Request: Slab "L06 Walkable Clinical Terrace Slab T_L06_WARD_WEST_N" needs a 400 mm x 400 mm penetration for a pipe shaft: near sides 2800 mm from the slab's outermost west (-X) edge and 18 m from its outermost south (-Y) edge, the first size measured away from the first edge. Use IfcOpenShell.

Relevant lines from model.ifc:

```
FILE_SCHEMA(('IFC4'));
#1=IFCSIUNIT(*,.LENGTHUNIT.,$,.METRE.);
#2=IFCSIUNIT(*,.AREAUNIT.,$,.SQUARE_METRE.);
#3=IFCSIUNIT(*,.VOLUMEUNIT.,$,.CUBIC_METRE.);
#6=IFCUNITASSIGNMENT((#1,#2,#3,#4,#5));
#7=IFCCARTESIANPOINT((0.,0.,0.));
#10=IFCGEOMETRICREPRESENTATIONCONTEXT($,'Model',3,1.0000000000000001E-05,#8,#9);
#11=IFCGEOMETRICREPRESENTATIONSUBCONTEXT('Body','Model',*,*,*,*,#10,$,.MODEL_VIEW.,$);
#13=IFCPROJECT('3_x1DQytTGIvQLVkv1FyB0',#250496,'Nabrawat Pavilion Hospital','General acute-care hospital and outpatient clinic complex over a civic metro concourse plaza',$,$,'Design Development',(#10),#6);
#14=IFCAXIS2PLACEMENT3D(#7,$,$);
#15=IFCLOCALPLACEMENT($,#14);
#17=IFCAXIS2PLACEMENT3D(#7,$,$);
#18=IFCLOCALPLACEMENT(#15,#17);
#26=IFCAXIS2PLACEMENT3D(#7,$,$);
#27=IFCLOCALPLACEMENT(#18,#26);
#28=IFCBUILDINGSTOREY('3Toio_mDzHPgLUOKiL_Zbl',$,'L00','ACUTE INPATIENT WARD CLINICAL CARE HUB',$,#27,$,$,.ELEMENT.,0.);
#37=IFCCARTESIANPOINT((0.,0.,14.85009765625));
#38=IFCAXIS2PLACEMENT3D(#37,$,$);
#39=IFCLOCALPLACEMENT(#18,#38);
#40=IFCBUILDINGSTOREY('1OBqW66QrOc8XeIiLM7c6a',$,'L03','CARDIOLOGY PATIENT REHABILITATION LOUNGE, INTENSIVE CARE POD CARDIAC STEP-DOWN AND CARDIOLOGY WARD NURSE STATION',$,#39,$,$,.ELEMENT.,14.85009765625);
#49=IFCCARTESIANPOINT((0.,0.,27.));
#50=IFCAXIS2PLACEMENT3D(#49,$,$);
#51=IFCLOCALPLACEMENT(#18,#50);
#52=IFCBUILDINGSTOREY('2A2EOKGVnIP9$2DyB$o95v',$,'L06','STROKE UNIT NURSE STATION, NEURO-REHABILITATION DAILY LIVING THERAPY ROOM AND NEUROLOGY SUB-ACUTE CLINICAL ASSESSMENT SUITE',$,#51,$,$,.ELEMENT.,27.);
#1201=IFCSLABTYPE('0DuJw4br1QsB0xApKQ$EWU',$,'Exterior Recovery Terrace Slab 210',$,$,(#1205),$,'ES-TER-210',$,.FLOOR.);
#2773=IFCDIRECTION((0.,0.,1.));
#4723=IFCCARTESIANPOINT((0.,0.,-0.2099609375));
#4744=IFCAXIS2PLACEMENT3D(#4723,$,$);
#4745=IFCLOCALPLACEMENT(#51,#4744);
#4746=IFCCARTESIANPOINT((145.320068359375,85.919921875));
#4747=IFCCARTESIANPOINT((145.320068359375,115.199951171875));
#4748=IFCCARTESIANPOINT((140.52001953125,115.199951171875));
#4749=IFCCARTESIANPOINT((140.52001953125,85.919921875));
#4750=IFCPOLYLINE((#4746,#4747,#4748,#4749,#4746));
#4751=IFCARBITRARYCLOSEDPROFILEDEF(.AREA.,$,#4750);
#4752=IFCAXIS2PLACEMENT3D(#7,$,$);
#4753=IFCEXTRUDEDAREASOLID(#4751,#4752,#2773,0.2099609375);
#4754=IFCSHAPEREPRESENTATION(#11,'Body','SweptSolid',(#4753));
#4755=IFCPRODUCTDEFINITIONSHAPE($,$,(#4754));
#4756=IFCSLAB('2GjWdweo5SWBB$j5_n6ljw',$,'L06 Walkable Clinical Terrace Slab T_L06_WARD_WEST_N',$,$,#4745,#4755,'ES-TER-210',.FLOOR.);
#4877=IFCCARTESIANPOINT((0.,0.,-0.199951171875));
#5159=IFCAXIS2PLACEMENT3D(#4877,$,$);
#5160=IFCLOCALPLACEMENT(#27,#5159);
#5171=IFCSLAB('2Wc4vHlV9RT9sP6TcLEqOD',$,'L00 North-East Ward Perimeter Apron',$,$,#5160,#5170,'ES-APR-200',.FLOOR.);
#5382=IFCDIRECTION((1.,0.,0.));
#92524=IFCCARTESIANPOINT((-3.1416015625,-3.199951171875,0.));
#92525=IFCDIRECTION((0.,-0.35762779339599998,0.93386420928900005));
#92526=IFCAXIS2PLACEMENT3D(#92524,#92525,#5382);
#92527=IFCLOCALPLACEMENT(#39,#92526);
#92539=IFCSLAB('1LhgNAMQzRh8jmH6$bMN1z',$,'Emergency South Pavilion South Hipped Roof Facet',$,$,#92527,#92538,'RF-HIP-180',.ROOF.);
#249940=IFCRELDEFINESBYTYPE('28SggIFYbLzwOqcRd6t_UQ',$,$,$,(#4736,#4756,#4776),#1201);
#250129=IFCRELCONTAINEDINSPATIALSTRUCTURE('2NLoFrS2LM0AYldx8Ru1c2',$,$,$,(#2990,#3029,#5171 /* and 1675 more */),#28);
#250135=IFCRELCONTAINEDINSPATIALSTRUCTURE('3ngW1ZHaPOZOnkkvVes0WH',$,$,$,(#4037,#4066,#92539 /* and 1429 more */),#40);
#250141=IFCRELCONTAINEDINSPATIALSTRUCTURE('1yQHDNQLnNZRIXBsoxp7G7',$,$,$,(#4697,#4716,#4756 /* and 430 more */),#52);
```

```python
import numpy as np
import ifcopenshell
import ifcopenshell.api.feature
import ifcopenshell.api.geometry
import ifcopenshell.api.root
import ifcopenshell.geom
import ifcopenshell.util.placement
import ifcopenshell.util.representation
import ifcopenshell.util.shape
import ifcopenshell.util.unit

model = ifcopenshell.open("model.ifc")
unit_scale = ifcopenshell.util.unit.calculate_unit_scale(model)
settings = ifcopenshell.geom.settings()


def volume(element):
    """Net volume in cubic metres, openings subtracted."""
    shape = ifcopenshell.geom.create_shape(settings, element)
    return ifcopenshell.util.shape.get_volume(shape.geometry)


slab = model.by_id(4756)
before = volume(slab)

# Extent in the slab's own axes, in metres. The edges named are its -X and -Y sides.
slab_shape = ifcopenshell.geom.create_shape(settings, slab)
vertices = ifcopenshell.util.shape.get_vertices(slab_shape.geometry)
x_min, y_min, bottom = vertices.min(axis=0)
top = vertices[:, 2].max()

opening = ifcopenshell.api.root.create_entity(model, ifc_class="IfcOpeningElement", name="Pipe shaft opening", predefined_type="OPENING")
context = ifcopenshell.util.representation.get_context(model, "Model", "Body", "MODEL_VIEW")
width, depth = 0.4, 0.4
outline = [(0.0, 0.0), (width, 0.0), (width, depth), (0.0, depth), (0.0, 0.0)]
# Overshoot both faces by 50 mm so the cut is clean.
shape = ifcopenshell.api.geometry.add_slab_representation(
    model, context=context, depth=top - bottom + 0.1, polyline=outline
)
ifcopenshell.api.geometry.assign_representation(model, product=opening, representation=shape)

matrix = ifcopenshell.util.placement.get_local_placement(slab.ObjectPlacement)
matrix[:, 3] = matrix @ np.append(np.array([x_min + 2.8, y_min + 18, bottom - 0.05]) / unit_scale, 1.0)
ifcopenshell.api.geometry.edit_object_placement(model, product=opening, matrix=matrix, is_si=False)
ifcopenshell.api.feature.add_feature(model, feature=opening, element=slab)

after = volume(slab)

print(f"slab volume {before:.3f} -> {after:.3f} m3")

model.write("model-out.ifc")
```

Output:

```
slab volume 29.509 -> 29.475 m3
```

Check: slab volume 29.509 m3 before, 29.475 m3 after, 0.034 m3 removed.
